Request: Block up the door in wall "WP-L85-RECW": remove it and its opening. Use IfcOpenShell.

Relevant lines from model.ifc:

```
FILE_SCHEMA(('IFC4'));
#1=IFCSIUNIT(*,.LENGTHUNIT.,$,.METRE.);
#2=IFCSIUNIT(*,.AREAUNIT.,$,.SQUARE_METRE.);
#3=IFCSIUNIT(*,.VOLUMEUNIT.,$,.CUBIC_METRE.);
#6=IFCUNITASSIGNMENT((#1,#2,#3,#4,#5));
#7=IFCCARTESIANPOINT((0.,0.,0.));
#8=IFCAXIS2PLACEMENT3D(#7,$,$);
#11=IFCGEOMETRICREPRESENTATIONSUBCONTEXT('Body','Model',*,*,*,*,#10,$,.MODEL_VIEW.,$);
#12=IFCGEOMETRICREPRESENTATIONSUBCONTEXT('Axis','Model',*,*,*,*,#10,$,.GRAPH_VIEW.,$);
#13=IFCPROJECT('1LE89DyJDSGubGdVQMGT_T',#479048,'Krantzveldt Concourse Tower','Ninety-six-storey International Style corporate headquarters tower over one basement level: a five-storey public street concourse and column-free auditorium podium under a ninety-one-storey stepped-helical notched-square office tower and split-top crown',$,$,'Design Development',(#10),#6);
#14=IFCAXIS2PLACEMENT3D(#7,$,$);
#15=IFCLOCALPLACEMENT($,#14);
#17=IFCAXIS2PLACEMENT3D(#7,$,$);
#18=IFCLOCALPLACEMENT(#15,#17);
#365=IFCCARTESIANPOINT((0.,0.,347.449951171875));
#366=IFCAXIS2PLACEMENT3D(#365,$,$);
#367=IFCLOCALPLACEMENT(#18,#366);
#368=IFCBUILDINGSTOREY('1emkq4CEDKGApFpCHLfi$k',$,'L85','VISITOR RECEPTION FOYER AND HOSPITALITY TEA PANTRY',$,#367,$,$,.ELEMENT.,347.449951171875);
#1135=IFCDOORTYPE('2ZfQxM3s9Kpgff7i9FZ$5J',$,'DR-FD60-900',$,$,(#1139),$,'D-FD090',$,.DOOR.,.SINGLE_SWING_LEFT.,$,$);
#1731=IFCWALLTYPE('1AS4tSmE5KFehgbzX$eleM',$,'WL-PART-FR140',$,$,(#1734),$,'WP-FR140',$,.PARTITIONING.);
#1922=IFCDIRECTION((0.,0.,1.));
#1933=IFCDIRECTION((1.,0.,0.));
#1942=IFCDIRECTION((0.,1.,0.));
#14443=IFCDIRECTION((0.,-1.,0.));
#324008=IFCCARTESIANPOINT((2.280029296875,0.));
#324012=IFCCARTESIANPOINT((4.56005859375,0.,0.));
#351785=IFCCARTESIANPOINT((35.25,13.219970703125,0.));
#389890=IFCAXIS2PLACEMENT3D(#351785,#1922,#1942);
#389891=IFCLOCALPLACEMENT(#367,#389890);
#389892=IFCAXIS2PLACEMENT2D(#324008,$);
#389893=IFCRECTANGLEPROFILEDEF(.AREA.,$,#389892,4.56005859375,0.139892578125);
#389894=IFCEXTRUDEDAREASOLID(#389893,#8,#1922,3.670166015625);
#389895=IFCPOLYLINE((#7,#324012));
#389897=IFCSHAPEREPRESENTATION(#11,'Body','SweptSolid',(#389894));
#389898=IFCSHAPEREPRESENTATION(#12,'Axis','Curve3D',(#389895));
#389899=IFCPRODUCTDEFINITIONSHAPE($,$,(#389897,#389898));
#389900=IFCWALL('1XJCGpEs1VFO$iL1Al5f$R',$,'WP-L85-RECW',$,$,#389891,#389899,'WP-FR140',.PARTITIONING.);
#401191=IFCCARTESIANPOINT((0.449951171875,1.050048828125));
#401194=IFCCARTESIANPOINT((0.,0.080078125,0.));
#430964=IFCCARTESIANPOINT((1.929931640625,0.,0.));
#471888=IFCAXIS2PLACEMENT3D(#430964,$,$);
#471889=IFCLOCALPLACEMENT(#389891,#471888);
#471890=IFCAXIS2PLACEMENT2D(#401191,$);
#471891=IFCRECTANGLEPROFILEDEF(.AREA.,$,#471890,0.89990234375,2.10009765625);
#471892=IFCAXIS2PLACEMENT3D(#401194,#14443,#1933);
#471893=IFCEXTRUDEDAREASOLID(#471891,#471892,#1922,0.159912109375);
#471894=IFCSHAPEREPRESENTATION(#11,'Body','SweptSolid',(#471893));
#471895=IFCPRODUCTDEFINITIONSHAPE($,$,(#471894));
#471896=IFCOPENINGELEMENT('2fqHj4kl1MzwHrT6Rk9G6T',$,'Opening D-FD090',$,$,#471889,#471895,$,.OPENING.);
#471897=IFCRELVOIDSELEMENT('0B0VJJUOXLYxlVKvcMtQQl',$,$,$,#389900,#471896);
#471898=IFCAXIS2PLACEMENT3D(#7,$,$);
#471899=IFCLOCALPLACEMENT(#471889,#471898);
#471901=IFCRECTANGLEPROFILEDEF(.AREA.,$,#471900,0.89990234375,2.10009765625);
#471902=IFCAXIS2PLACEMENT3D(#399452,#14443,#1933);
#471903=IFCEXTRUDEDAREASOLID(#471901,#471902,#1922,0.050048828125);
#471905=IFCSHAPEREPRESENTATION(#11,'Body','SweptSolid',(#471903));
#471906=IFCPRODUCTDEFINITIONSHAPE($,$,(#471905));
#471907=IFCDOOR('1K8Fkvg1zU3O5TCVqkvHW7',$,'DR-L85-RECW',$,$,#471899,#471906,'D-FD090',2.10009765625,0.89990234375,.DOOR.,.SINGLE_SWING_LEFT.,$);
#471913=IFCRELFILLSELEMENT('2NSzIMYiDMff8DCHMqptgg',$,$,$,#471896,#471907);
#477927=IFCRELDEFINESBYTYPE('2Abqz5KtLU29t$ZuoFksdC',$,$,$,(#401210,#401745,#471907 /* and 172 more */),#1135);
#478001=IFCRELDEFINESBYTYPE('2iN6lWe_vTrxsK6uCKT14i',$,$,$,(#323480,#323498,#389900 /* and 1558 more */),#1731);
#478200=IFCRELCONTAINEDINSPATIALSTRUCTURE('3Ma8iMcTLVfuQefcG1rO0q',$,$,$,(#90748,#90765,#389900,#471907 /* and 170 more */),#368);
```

```python
import ifcopenshell
import ifcopenshell.api.feature
import ifcopenshell.api.root
import ifcopenshell.geom
import ifcopenshell.util.shape

model = ifcopenshell.open("model.ifc")
settings = ifcopenshell.geom.settings()


def volume(element):
    """Net volume in cubic metres, openings subtracted."""
    shape = ifcopenshell.geom.create_shape(settings, element)
    return ifcopenshell.util.shape.get_volume(shape.geometry)


door = model.by_guid("1K8Fkvg1zU3O5TCVqkvHW7")
opening = door.FillsVoids[0].RelatingOpeningElement
wall = opening.VoidsElements[0].RelatingBuildingElement
before = volume(wall)

ifcopenshell.api.root.remove_product(model, product=door)
ifcopenshell.api.feature.remove_feature(model, feature=opening)

after = volume(wall)

print(f"wall volume {before:.3f} -> {after:.3f} m3")

model.write("model_rev.ifc")
```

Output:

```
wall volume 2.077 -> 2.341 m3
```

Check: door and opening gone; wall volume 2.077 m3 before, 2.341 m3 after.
